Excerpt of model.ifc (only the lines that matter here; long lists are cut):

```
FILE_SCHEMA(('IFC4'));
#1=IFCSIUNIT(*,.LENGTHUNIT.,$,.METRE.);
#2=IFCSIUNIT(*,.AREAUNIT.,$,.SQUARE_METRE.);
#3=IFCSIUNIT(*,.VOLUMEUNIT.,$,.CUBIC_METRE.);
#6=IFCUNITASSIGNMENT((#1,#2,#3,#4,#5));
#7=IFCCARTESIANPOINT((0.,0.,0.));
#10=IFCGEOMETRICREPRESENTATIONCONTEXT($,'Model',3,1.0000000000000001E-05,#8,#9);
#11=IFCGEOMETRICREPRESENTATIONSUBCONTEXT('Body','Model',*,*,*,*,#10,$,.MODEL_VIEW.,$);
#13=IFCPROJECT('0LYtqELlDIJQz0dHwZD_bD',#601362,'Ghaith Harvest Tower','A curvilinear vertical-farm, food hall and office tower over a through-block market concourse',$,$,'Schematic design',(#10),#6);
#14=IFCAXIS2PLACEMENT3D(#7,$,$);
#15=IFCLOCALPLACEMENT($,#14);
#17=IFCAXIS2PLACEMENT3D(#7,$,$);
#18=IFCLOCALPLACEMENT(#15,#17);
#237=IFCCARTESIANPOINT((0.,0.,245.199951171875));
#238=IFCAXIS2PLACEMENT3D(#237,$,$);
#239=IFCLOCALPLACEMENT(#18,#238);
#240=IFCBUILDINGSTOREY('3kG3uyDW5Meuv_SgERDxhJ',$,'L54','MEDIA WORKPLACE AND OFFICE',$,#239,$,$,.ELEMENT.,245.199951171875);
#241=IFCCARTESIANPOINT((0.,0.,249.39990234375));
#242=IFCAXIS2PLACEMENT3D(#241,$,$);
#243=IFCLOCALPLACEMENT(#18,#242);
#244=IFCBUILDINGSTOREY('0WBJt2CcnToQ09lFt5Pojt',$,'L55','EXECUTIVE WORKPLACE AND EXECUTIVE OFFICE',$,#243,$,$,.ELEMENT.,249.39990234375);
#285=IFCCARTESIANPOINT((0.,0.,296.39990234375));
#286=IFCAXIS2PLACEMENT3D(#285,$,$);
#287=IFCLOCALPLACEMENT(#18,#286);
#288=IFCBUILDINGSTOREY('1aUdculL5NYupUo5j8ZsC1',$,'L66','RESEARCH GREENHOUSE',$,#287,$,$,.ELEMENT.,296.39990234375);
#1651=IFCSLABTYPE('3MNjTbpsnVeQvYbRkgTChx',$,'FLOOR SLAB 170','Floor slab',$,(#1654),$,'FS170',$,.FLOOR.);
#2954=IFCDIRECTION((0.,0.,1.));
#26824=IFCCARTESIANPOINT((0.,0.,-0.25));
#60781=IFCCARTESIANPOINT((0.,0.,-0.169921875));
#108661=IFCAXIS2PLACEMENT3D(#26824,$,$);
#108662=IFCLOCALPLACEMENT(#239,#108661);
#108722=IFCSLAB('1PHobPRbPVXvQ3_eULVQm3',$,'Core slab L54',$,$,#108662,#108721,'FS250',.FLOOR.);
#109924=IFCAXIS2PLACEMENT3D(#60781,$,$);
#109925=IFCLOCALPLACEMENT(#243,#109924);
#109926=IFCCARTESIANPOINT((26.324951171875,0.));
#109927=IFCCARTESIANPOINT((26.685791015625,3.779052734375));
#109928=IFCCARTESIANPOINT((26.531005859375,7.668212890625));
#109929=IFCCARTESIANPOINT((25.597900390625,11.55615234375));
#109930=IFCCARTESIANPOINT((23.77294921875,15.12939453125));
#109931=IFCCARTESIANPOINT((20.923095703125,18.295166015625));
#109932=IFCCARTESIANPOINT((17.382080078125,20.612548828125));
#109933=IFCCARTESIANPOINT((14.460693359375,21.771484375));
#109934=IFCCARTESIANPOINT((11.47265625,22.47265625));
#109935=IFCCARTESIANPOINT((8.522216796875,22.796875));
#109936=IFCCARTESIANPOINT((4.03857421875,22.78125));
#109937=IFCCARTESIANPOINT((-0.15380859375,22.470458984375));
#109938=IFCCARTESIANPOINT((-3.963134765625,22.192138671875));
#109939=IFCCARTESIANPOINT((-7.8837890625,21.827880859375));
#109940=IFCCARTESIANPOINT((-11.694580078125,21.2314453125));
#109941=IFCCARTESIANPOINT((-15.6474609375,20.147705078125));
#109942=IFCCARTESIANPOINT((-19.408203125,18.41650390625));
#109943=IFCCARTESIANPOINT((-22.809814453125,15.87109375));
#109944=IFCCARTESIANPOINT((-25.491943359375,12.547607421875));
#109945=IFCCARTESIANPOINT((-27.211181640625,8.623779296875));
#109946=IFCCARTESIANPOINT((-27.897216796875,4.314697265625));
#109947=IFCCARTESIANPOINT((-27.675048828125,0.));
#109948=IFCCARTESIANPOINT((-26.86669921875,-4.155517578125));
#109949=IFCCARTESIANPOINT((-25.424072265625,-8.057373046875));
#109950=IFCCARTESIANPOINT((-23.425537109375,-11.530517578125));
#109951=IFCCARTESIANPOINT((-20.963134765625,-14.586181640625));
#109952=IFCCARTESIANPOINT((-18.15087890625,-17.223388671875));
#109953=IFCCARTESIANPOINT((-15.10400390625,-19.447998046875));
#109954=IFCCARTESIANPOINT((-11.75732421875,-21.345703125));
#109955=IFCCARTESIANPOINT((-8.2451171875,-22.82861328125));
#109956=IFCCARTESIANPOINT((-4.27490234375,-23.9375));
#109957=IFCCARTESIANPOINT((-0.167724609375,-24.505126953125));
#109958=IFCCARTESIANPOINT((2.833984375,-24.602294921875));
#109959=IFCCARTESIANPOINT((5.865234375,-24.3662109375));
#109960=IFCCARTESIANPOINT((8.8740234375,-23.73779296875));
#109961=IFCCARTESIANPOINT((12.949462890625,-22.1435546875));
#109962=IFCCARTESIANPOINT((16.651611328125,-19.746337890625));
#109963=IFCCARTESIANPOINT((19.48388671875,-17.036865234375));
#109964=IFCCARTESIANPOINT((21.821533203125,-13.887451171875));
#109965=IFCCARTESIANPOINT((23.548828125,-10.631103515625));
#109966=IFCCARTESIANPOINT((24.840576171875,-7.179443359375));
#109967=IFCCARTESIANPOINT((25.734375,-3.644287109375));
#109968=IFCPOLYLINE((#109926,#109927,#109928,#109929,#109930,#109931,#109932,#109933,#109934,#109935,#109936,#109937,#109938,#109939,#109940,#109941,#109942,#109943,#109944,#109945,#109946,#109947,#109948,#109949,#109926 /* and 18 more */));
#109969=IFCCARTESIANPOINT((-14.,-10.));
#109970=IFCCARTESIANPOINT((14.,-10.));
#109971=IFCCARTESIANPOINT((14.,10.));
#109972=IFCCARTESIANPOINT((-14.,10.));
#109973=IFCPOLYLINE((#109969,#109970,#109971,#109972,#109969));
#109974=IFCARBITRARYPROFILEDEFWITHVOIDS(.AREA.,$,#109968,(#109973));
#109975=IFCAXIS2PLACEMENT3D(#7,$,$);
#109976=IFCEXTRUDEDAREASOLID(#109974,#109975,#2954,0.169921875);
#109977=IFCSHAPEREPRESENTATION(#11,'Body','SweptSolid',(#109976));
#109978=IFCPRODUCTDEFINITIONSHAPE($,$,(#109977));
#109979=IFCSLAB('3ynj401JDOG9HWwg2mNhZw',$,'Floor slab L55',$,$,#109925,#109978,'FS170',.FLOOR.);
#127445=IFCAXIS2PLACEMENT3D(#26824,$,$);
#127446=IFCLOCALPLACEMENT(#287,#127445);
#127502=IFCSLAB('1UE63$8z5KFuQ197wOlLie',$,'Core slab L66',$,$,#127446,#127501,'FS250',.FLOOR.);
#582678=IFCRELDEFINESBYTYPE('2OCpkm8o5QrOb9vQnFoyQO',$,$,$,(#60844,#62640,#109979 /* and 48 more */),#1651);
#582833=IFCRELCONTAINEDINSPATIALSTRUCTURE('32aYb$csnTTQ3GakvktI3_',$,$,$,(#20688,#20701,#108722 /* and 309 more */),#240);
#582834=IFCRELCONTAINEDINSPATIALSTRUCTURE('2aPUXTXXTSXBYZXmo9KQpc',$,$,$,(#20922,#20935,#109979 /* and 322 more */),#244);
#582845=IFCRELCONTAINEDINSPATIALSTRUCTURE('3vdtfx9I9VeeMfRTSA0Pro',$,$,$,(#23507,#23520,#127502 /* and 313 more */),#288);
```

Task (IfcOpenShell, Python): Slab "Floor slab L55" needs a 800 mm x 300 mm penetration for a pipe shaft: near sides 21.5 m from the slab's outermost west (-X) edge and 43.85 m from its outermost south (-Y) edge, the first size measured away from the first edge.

```python
import numpy as np
import ifcopenshell
import ifcopenshell.api.feature
import ifcopenshell.api.geometry
import ifcopenshell.api.root
import ifcopenshell.geom
import ifcopenshell.util.placement
import ifcopenshell.util.representation
import ifcopenshell.util.shape
import ifcopenshell.util.unit

model = ifcopenshell.open("model.ifc")
unit_scale = ifcopenshell.util.unit.calculate_unit_scale(model)
settings = ifcopenshell.geom.settings()


def volume(element):
    """Net volume in cubic metres, openings subtracted."""
    shape = ifcopenshell.geom.create_shape(settings, element)
    return ifcopenshell.util.shape.get_volume(shape.geometry)


slab = model.by_guid("3ynj401JDOG9HWwg2mNhZw")
before = volume(slab)

# Extent in the slab's own axes, in metres. The edges named are its -X and -Y sides.
slab_shape = ifcopenshell.geom.create_shape(settings, slab)
vertices = ifcopenshell.util.shape.get_vertices(slab_shape.geometry)
x_min, y_min, bottom = vertices.min(axis=0)
top = vertices[:, 2].max()

opening = ifcopenshell.api.root.create_entity(model, ifc_class="IfcOpeningElement", name="Pipe shaft opening", predefined_type="OPENING")
context = ifcopenshell.util.representation.get_context(model, "Model", "Body", "MODEL_VIEW")
width, depth = 0.8, 0.3
outline = [(0.0, 0.0), (width, 0.0), (width, depth), (0.0, depth), (0.0, 0.0)]
# Overshoot both faces by 50 mm so the cut is clean.
shape = ifcopenshell.api.geometry.add_slab_representation(
    model, context=context, depth=top - bottom + 0.1, polyline=outline
)
ifcopenshell.api.geometry.assign_representation(model, product=opening, representation=shape)

matrix = ifcopenshell.util.placement.get_local_placement(slab.ObjectPlacement)
matrix[:, 3] = matrix @ np.append(np.array([x_min + 21.5, y_min + 43.85, bottom - 0.05]) / unit_scale, 1.0)
ifcopenshell.api.geometry.edit_object_placement(model, product=opening, matrix=matrix, is_si=False)
ifcopenshell.api.feature.add_feature(model, feature=opening, element=slab)

after = volume(slab)

print(f"slab volume {before:.3f} -> {after:.3f} m3")

model.write("model_rev.ifc")
```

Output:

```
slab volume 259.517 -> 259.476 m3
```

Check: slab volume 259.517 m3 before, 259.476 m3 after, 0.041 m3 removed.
